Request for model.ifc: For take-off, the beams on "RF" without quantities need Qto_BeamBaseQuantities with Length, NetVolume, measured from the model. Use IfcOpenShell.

First a look at what the model holds.

```python
import ifcopenshell
import ifcopenshell.util.element
import ifcopenshell.util.unit

model = ifcopenshell.open("model.ifc")
print(model.schema)
for unit_type in ("LENGTHUNIT", "AREAUNIT", "VOLUMEUNIT"):
    print(unit_type, ifcopenshell.util.unit.calculate_unit_scale(model, unit_type))
storey = next(s for s in model.by_type("IfcBuildingStorey") if s.Name == "RF")
beams = [e for e in ifcopenshell.util.element.get_decomposition(storey) if e.is_a("IfcBeam")]
for e in sorted(beams, key=lambda e: e.id()):
    print(e.id(), e.is_a(), e.Name, list(ifcopenshell.util.element.get_psets(e, qtos_only=True)), sep=" | ")
```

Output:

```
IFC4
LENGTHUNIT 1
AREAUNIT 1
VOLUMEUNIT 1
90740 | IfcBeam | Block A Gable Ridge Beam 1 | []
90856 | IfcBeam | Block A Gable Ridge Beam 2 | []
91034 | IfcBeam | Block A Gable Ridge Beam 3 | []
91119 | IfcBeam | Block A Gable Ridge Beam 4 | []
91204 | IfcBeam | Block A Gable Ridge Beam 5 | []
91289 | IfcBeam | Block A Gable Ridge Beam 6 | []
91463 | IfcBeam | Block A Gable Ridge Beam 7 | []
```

```python
import ifcopenshell
import ifcopenshell.api.pset
import ifcopenshell.geom
import ifcopenshell.util.element
import ifcopenshell.util.shape
import ifcopenshell.util.unit

model = ifcopenshell.open("model.ifc")
unit_scale = ifcopenshell.util.unit.calculate_unit_scale(model)
volume_scale = ifcopenshell.util.unit.calculate_unit_scale(model, "VOLUMEUNIT")
settings = ifcopenshell.geom.settings()

storey = next(s for s in model.by_type("IfcBuildingStorey") if s.Name == "RF")
beams = [e for e in ifcopenshell.util.element.get_decomposition(storey) if e.is_a("IfcBeam")]

for e in sorted(beams, key=lambda e: e.id()):
    if ifcopenshell.util.element.get_psets(e, qtos_only=True, should_inherit=False):
        continue
    # Geometry comes back in metres, in the element's own axes.
    shape = ifcopenshell.geom.create_shape(settings, e)
    values = {
        "Length": ifcopenshell.util.shape.get_max_xyz(shape.geometry) / unit_scale,
        "NetVolume": ifcopenshell.util.shape.get_volume(shape.geometry) / volume_scale,
    }
    qto = ifcopenshell.api.pset.add_qto(model, product=e, name="Qto_BeamBaseQuantities")
    ifcopenshell.api.pset.edit_qto(model, qto=qto, properties=values)
    print(e.id(), {k: round(v, 3) for k, v in values.items()})

model.write("model_edited.ifc")
```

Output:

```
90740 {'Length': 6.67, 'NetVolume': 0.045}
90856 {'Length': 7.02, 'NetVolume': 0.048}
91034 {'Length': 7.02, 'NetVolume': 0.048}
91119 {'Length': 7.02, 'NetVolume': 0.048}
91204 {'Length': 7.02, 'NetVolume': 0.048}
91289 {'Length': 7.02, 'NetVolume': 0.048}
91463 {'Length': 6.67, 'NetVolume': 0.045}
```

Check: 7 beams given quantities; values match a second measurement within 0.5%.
